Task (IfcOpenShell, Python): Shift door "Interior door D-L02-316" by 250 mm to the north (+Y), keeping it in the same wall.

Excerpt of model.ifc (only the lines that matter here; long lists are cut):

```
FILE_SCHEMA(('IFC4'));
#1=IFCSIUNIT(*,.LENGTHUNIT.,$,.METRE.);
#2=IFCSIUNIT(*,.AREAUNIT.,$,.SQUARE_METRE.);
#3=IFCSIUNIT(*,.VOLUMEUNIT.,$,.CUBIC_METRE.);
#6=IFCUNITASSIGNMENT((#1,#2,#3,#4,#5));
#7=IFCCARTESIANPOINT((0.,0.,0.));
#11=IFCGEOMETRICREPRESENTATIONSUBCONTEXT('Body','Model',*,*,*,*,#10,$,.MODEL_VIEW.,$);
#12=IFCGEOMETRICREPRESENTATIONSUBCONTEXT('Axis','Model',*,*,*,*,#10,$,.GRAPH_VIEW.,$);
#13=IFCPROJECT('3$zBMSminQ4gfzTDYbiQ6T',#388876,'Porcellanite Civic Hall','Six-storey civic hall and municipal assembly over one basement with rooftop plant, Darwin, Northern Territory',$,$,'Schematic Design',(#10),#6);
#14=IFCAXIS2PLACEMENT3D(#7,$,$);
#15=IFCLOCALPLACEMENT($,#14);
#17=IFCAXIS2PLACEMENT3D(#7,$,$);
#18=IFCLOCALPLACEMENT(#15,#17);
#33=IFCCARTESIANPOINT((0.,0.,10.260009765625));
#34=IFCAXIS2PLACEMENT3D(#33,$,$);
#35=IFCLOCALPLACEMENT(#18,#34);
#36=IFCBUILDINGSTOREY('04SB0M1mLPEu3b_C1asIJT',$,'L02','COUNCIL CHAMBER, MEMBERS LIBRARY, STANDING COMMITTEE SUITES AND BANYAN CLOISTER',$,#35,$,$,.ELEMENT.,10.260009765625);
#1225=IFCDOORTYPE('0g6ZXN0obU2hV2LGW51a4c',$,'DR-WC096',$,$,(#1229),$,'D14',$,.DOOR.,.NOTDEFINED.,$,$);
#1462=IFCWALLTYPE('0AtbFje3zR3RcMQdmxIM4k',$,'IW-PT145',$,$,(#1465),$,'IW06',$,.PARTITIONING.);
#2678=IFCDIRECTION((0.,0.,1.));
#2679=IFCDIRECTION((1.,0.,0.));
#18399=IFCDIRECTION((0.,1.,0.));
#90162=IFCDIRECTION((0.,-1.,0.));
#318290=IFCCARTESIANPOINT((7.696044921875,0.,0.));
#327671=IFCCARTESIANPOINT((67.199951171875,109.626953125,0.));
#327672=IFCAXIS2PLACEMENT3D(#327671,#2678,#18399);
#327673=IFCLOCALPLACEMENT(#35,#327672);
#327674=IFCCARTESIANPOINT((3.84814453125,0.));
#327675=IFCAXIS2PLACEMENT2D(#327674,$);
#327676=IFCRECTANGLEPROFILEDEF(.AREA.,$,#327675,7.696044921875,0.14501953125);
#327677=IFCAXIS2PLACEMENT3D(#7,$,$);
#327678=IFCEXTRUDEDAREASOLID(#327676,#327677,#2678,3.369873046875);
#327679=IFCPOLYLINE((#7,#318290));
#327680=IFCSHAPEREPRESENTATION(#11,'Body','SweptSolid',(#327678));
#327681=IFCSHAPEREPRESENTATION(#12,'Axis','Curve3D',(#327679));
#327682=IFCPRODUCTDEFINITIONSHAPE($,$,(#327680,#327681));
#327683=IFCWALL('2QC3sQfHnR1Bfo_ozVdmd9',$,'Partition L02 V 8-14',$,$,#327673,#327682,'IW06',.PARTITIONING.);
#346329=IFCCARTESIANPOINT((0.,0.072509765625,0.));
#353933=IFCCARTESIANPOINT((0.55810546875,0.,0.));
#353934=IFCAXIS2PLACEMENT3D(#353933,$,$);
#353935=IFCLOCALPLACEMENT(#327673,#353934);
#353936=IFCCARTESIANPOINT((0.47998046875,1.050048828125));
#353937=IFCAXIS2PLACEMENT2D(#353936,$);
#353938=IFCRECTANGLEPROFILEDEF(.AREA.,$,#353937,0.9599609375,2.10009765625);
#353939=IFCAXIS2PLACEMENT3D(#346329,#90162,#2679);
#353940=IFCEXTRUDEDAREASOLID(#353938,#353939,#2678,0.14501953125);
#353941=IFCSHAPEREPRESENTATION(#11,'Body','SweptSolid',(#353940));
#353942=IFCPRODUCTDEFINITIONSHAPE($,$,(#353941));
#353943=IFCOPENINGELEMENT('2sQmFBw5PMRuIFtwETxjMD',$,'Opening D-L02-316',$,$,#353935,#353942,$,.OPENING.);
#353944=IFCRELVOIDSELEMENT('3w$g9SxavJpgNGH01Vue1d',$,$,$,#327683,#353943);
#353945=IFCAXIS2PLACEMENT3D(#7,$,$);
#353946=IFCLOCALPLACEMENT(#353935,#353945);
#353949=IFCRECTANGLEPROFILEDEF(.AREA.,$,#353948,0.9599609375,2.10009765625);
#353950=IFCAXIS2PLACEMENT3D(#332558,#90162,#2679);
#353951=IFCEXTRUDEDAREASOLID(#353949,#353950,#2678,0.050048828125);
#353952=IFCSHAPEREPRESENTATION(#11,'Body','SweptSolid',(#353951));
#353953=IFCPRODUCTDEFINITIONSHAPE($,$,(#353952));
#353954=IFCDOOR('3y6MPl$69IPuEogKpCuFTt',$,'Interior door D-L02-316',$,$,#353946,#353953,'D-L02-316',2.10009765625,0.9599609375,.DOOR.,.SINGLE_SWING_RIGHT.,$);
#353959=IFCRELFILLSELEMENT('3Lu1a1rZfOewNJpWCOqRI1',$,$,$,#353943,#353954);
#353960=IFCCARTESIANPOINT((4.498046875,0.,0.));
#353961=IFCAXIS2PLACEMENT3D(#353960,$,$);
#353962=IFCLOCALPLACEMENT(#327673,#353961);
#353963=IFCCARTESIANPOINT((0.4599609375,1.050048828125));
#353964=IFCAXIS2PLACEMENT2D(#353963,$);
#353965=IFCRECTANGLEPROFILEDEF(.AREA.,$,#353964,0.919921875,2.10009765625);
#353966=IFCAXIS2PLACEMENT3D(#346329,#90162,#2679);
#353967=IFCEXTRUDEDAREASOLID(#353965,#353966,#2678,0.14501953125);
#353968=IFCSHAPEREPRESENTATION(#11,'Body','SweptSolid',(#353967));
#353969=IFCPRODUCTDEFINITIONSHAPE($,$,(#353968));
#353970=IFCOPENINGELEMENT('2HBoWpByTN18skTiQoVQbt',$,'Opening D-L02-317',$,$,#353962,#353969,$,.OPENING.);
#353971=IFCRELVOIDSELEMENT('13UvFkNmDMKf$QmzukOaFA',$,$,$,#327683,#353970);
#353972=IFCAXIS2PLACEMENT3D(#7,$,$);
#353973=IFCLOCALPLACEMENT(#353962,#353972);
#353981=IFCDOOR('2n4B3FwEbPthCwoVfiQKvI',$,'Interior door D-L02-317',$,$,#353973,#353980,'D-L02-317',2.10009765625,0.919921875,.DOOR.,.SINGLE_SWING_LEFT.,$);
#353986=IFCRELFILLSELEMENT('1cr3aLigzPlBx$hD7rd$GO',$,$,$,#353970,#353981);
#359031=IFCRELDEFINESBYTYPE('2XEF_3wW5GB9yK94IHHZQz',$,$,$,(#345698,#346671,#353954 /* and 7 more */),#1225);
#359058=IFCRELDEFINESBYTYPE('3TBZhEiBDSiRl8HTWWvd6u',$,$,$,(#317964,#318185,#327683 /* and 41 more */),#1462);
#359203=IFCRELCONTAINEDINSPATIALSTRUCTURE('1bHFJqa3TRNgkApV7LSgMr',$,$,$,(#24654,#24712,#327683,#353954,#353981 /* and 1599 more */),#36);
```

```python
import ifcopenshell
import ifcopenshell.api.geometry
import ifcopenshell.util.placement

model = ifcopenshell.open("model.ifc")

door = model.by_guid("3y6MPl$69IPuEogKpCuFTt")
opening = door.FillsVoids[0].RelatingOpeningElement
wall = opening.VoidsElements[0].RelatingBuildingElement

wall_matrix = ifcopenshell.util.placement.get_local_placement(wall.ObjectPlacement)
shift = wall_matrix[:3, 0] * 0.25
before = ifcopenshell.util.placement.get_local_placement(door.ObjectPlacement)[:3, 3].copy()

# The door is placed relative to its opening, so it follows when the opening moves.
matrix = ifcopenshell.util.placement.get_local_placement(opening.ObjectPlacement)
matrix[:3, 3] += shift
ifcopenshell.api.geometry.edit_object_placement(
    model, product=opening, matrix=matrix, is_si=False, should_transform_children=True
)

after = ifcopenshell.util.placement.get_local_placement(door.ObjectPlacement)[:3, 3]
print("door moved by", (after - before).round(3) + 0.0)

model.write("model_updated.ifc")
```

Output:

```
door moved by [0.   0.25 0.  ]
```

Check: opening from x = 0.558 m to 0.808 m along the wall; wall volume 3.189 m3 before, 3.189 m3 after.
